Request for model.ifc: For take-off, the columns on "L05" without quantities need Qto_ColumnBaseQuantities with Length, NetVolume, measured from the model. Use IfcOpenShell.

First a look at what the model holds.

```python
import ifcopenshell
import ifcopenshell.util.element
import ifcopenshell.util.unit

model = ifcopenshell.open("model.ifc")
print(model.schema)
for unit_type in ("LENGTHUNIT", "AREAUNIT", "VOLUMEUNIT"):
    print(unit_type, ifcopenshell.util.unit.calculate_unit_scale(model, unit_type))
storey = next(s for s in model.by_type("IfcBuildingStorey") if s.Name == "L05")
columns = [e for e in ifcopenshell.util.element.get_decomposition(storey) if e.is_a("IfcColumn")]
for e in sorted(columns, key=lambda e: e.id()):
    print(e.id(), e.is_a(), e.Name, list(ifcopenshell.util.element.get_psets(e, qtos_only=True)), sep=" | ")
```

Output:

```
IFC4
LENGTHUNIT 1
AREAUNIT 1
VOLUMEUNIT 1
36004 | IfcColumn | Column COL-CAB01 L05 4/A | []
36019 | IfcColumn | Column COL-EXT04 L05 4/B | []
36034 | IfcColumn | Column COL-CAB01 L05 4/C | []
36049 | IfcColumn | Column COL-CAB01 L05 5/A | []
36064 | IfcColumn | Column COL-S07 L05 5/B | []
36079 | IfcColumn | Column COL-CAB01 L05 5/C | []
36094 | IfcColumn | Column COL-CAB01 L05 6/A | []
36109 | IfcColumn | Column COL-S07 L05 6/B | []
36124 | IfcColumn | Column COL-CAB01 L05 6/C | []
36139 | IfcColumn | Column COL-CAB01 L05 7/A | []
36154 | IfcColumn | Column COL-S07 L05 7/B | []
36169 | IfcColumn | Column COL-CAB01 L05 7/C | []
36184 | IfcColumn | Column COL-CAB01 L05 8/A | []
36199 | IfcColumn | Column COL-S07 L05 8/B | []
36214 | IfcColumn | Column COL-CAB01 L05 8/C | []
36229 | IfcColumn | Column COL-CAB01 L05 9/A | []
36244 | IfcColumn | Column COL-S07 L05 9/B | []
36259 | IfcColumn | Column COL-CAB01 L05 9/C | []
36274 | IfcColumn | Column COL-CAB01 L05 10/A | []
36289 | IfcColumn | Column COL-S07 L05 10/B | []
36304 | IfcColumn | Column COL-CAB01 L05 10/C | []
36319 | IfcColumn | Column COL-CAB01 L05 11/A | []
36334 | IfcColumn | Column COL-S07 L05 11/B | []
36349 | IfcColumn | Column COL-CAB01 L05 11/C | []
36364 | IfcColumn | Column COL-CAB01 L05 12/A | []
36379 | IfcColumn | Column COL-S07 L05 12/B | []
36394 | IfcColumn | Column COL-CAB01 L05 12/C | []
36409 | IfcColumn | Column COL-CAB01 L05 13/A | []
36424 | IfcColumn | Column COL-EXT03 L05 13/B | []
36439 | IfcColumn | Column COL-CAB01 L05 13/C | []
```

```python
import ifcopenshell
import ifcopenshell.api.pset
import ifcopenshell.geom
import ifcopenshell.util.element
import ifcopenshell.util.shape
import ifcopenshell.util.unit

model = ifcopenshell.open("model.ifc")
unit_scale = ifcopenshell.util.unit.calculate_unit_scale(model)
volume_scale = ifcopenshell.util.unit.calculate_unit_scale(model, "VOLUMEUNIT")
settings = ifcopenshell.geom.settings()

storey = next(s for s in model.by_type("IfcBuildingStorey") if s.Name == "L05")
columns = [e for e in ifcopenshell.util.element.get_decomposition(storey) if e.is_a("IfcColumn")]

for e in sorted(columns, key=lambda e: e.id()):
    if ifcopenshell.util.element.get_psets(e, qtos_only=True, should_inherit=False):
        continue
    # Geometry comes back in metres, in the element's own axes.
    shape = ifcopenshell.geom.create_shape(settings, e)
    values = {
        "Length": ifcopenshell.util.shape.get_z(shape.geometry) / unit_scale,
        "NetVolume": ifcopenshell.util.shape.get_volume(shape.geometry) / volume_scale,
    }
    qto = ifcopenshell.api.pset.add_qto(model, product=e, name="Qto_ColumnBaseQuantities")
    ifcopenshell.api.pset.edit_qto(model, qto=qto, properties=values)
    print(e.id(), {k: round(v, 3) for k, v in values.items()})

model.write("model_rev.ifc")
```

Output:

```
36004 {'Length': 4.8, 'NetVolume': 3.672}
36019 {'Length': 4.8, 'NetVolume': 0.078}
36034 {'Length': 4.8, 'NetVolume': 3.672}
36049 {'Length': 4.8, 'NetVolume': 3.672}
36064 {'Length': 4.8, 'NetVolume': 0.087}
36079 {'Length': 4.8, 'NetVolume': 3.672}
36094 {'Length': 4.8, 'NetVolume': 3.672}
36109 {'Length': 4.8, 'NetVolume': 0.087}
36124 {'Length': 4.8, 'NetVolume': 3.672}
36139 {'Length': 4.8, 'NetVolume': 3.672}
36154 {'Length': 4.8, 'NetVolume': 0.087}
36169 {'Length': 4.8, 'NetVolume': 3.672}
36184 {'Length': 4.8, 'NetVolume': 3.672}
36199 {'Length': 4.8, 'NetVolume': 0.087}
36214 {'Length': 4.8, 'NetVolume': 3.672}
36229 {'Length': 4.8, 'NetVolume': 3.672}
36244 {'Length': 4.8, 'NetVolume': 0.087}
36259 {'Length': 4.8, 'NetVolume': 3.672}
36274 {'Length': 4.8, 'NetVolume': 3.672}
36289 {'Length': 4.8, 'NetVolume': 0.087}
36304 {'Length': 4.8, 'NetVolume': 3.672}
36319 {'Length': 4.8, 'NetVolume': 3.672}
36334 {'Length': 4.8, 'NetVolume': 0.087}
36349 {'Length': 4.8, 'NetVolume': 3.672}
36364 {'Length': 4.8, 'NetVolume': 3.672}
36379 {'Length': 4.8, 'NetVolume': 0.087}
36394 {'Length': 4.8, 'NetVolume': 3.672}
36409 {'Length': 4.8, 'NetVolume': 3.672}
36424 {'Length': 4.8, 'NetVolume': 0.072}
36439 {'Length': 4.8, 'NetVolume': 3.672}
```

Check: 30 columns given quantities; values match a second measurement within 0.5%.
